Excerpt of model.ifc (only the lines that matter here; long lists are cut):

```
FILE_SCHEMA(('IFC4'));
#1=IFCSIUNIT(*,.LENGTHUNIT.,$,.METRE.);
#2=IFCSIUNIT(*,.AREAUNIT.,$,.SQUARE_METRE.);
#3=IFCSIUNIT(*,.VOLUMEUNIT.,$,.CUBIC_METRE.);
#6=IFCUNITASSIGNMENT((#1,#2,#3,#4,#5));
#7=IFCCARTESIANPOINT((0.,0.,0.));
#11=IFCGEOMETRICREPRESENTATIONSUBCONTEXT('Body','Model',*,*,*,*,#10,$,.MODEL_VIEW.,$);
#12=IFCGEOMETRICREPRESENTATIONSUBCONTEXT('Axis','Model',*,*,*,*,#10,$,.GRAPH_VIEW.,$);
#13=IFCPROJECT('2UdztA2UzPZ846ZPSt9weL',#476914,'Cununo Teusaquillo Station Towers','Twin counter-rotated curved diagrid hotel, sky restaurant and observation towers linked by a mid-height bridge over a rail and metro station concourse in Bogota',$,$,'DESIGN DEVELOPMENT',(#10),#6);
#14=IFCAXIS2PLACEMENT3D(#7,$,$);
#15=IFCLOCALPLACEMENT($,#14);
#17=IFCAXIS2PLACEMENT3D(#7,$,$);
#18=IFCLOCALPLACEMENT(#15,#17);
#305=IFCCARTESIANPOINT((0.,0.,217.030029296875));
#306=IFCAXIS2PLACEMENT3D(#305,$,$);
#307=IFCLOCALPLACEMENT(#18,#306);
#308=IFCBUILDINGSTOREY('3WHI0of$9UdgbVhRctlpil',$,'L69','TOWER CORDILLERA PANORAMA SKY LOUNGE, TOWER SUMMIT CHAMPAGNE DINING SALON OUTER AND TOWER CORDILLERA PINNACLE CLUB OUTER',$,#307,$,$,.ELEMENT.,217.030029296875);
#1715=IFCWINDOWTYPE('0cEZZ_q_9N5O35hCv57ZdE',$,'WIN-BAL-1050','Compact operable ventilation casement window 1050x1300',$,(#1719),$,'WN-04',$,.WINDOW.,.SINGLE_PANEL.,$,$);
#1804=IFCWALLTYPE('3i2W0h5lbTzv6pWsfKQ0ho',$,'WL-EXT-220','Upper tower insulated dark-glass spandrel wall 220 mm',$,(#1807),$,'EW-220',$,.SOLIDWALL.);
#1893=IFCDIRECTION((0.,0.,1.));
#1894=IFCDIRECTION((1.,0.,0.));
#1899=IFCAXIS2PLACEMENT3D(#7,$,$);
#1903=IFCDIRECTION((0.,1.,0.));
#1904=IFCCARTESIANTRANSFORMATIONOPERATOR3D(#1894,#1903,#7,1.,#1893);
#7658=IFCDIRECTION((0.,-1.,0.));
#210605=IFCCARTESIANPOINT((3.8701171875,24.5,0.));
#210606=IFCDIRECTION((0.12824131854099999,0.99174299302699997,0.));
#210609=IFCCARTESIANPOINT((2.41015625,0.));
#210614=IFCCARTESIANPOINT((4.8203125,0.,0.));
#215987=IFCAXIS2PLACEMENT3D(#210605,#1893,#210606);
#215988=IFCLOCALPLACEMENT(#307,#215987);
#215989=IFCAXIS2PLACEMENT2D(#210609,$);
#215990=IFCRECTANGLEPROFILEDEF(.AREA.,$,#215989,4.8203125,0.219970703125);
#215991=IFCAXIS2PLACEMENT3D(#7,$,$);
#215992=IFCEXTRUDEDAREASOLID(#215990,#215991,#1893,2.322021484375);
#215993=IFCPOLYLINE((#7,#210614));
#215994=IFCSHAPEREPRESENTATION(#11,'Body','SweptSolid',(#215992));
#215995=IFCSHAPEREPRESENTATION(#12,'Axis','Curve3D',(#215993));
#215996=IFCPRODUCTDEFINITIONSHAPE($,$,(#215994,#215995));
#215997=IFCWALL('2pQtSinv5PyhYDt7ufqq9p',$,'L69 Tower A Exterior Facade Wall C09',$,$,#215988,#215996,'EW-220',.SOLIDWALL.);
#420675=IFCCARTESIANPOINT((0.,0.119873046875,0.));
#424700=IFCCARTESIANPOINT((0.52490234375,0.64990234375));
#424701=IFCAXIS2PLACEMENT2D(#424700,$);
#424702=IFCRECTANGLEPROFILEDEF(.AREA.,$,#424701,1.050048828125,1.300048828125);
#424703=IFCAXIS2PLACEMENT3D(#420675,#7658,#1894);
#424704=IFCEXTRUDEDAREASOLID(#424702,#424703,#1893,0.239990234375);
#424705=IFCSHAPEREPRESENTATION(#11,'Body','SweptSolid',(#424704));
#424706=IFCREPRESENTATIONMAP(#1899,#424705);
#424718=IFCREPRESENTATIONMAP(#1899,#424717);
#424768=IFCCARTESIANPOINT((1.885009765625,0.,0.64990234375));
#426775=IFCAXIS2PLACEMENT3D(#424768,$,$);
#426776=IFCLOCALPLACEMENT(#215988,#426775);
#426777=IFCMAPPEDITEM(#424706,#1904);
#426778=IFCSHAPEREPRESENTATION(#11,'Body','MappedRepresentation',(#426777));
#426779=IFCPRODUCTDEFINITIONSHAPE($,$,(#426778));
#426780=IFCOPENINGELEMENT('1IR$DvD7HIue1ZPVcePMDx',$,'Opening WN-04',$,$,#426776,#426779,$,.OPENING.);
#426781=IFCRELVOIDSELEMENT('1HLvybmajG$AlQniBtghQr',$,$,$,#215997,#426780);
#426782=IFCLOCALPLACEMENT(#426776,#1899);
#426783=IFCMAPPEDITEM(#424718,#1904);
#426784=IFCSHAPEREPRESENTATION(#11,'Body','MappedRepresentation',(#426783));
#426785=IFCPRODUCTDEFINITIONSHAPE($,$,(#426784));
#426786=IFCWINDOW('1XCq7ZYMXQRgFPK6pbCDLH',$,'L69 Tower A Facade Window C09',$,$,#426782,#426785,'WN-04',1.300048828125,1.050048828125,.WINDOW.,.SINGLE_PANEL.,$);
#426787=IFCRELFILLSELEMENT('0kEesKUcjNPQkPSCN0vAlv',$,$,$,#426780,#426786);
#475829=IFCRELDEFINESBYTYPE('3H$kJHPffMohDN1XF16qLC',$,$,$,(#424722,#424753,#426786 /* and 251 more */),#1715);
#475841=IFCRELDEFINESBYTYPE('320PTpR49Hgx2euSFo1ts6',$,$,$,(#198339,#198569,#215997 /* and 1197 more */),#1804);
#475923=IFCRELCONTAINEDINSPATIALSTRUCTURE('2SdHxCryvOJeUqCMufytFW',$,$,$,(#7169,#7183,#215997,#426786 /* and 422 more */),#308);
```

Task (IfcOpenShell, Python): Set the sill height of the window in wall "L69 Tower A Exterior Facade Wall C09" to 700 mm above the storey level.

```python
import numpy as np
import ifcopenshell
import ifcopenshell.api.geometry
import ifcopenshell.geom
import ifcopenshell.util.element
import ifcopenshell.util.placement
import ifcopenshell.util.shape
import ifcopenshell.util.unit

model = ifcopenshell.open("model.ifc")
unit_scale = ifcopenshell.util.unit.calculate_unit_scale(model)

window = model.by_id(426786)
opening = window.FillsVoids[0].RelatingOpeningElement
storey = ifcopenshell.util.element.get_container(window, ifc_class="IfcBuildingStorey")
level = ifcopenshell.util.placement.get_local_placement(storey.ObjectPlacement)[2, 3]

# The opening's origin need not be at the sill, so measure its lowest point.
shape = ifcopenshell.geom.create_shape(ifcopenshell.geom.settings(), opening)
bottom = ifcopenshell.util.shape.get_shape_bottom_elevation(shape, shape.geometry) / unit_scale
dz = level + 0.7 / unit_scale - bottom

shift = np.array([0.0, 0.0, dz])
# The window is placed relative to its opening, so it follows when the opening moves.
matrix = ifcopenshell.util.placement.get_local_placement(opening.ObjectPlacement)
matrix[:3, 3] += shift
ifcopenshell.api.geometry.edit_object_placement(
    model, product=opening, matrix=matrix, is_si=False, should_transform_children=True
)

print(f"moved by {dz * unit_scale:+.3f} m")

model.write("model_edited.ifc")
```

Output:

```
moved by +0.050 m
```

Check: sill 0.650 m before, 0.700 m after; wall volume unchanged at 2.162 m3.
